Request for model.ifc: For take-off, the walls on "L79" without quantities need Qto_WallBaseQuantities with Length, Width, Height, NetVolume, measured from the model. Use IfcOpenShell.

First a look at what the model holds.

```python
import ifcopenshell
import ifcopenshell.util.element
import ifcopenshell.util.unit

model = ifcopenshell.open("model.ifc")
print(model.schema)
for unit_type in ("LENGTHUNIT", "AREAUNIT", "VOLUMEUNIT"):
    print(unit_type, ifcopenshell.util.unit.calculate_unit_scale(model, unit_type))
storey = next(s for s in model.by_type("IfcBuildingStorey") if s.Name == "L79")
walls = [e for e in ifcopenshell.util.element.get_decomposition(storey) if e.is_a("IfcWall")]
for e in sorted(walls, key=lambda e: e.id()):
    print(e.id(), e.is_a(), e.Name, list(ifcopenshell.util.element.get_psets(e, qtos_only=True)), sep=" | ")
```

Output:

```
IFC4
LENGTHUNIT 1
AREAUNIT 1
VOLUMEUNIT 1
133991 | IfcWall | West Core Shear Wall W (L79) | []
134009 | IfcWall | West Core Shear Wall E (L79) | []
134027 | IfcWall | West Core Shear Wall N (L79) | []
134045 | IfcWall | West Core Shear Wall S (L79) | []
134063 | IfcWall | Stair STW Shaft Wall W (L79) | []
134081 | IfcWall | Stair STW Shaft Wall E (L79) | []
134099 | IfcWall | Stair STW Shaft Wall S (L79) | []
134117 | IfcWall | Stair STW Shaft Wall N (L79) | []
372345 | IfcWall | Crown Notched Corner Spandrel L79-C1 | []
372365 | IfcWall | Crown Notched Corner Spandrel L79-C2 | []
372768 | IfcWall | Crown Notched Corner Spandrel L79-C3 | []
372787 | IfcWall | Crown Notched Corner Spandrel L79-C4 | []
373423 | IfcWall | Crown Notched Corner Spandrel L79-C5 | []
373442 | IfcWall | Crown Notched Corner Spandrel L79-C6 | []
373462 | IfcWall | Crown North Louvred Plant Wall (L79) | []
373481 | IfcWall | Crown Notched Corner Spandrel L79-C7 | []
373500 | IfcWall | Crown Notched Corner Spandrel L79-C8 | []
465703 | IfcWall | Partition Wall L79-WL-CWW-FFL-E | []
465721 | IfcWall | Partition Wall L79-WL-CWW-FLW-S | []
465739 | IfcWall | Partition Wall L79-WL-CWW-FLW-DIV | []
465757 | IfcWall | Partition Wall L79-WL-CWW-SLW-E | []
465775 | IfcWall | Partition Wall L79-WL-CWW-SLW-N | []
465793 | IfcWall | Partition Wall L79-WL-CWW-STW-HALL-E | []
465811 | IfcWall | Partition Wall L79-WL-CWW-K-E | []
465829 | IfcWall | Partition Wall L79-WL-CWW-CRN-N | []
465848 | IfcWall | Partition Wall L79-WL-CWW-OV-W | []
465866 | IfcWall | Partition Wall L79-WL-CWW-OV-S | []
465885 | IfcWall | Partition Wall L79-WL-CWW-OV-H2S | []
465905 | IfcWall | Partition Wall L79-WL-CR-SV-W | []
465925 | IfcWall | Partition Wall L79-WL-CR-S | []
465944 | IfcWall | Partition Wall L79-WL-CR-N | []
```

```python
import ifcopenshell
import ifcopenshell.api.pset
import ifcopenshell.geom
import ifcopenshell.util.element
import ifcopenshell.util.shape
import ifcopenshell.util.unit

model = ifcopenshell.open("model.ifc")
unit_scale = ifcopenshell.util.unit.calculate_unit_scale(model)
volume_scale = ifcopenshell.util.unit.calculate_unit_scale(model, "VOLUMEUNIT")
settings = ifcopenshell.geom.settings()

storey = next(s for s in model.by_type("IfcBuildingStorey") if s.Name == "L79")
walls = [e for e in ifcopenshell.util.element.get_decomposition(storey) if e.is_a("IfcWall")]

for e in sorted(walls, key=lambda e: e.id()):
    if ifcopenshell.util.element.get_psets(e, qtos_only=True, should_inherit=False):
        continue
    # Geometry comes back in metres, in the element's own axes.
    shape = ifcopenshell.geom.create_shape(settings, e)
    values = {
        "Length": ifcopenshell.util.shape.get_x(shape.geometry) / unit_scale,
        "Width": ifcopenshell.util.shape.get_y(shape.geometry) / unit_scale,
        "Height": ifcopenshell.util.shape.get_z(shape.geometry) / unit_scale,
        "NetVolume": ifcopenshell.util.shape.get_volume(shape.geometry) / volume_scale,
    }
    qto = ifcopenshell.api.pset.add_qto(model, product=e, name="Qto_WallBaseQuantities")
    ifcopenshell.api.pset.edit_qto(model, qto=qto, properties=values)
    print(e.id(), {k: round(v, 3) for k, v in values.items()})

model.write("model-out.ifc")
```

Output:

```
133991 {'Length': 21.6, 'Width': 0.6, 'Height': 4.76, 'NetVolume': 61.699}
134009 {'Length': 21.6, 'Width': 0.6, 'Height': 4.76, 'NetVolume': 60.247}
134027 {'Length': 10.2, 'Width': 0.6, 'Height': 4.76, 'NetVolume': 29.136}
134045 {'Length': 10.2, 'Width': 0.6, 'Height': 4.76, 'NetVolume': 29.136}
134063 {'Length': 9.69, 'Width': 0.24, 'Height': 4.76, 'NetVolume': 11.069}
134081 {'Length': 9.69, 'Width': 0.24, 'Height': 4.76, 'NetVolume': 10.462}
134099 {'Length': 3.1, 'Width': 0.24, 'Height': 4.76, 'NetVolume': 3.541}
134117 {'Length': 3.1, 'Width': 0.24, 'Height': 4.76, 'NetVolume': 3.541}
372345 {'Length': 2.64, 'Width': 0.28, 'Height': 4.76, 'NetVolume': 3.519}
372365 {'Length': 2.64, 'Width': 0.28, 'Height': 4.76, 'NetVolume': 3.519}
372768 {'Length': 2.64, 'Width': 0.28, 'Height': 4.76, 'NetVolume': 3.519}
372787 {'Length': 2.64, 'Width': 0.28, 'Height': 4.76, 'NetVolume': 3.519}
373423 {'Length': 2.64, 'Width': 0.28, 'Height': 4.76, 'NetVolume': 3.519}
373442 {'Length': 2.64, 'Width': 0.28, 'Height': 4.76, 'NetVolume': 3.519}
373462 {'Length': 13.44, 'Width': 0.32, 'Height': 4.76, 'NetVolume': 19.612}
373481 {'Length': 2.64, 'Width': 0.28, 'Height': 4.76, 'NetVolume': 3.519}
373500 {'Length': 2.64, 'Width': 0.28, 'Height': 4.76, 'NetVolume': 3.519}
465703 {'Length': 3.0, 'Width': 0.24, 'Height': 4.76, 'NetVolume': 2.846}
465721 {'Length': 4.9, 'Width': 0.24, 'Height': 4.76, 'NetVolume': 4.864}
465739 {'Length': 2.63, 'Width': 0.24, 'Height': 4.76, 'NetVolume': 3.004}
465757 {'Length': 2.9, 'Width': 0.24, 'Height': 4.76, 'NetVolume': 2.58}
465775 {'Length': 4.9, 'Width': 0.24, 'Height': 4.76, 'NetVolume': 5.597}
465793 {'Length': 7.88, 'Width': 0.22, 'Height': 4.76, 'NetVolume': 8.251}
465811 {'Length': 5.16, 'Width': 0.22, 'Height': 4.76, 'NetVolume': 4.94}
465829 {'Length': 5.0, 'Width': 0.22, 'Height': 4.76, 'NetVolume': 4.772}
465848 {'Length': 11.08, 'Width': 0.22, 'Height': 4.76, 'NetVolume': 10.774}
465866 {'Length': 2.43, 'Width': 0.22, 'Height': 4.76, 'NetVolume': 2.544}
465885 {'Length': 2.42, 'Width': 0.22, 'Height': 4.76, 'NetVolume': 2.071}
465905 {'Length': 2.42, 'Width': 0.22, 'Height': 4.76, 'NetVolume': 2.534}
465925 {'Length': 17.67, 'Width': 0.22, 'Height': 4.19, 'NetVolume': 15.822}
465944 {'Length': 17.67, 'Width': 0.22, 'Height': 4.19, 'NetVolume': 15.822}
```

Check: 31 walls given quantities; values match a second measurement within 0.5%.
